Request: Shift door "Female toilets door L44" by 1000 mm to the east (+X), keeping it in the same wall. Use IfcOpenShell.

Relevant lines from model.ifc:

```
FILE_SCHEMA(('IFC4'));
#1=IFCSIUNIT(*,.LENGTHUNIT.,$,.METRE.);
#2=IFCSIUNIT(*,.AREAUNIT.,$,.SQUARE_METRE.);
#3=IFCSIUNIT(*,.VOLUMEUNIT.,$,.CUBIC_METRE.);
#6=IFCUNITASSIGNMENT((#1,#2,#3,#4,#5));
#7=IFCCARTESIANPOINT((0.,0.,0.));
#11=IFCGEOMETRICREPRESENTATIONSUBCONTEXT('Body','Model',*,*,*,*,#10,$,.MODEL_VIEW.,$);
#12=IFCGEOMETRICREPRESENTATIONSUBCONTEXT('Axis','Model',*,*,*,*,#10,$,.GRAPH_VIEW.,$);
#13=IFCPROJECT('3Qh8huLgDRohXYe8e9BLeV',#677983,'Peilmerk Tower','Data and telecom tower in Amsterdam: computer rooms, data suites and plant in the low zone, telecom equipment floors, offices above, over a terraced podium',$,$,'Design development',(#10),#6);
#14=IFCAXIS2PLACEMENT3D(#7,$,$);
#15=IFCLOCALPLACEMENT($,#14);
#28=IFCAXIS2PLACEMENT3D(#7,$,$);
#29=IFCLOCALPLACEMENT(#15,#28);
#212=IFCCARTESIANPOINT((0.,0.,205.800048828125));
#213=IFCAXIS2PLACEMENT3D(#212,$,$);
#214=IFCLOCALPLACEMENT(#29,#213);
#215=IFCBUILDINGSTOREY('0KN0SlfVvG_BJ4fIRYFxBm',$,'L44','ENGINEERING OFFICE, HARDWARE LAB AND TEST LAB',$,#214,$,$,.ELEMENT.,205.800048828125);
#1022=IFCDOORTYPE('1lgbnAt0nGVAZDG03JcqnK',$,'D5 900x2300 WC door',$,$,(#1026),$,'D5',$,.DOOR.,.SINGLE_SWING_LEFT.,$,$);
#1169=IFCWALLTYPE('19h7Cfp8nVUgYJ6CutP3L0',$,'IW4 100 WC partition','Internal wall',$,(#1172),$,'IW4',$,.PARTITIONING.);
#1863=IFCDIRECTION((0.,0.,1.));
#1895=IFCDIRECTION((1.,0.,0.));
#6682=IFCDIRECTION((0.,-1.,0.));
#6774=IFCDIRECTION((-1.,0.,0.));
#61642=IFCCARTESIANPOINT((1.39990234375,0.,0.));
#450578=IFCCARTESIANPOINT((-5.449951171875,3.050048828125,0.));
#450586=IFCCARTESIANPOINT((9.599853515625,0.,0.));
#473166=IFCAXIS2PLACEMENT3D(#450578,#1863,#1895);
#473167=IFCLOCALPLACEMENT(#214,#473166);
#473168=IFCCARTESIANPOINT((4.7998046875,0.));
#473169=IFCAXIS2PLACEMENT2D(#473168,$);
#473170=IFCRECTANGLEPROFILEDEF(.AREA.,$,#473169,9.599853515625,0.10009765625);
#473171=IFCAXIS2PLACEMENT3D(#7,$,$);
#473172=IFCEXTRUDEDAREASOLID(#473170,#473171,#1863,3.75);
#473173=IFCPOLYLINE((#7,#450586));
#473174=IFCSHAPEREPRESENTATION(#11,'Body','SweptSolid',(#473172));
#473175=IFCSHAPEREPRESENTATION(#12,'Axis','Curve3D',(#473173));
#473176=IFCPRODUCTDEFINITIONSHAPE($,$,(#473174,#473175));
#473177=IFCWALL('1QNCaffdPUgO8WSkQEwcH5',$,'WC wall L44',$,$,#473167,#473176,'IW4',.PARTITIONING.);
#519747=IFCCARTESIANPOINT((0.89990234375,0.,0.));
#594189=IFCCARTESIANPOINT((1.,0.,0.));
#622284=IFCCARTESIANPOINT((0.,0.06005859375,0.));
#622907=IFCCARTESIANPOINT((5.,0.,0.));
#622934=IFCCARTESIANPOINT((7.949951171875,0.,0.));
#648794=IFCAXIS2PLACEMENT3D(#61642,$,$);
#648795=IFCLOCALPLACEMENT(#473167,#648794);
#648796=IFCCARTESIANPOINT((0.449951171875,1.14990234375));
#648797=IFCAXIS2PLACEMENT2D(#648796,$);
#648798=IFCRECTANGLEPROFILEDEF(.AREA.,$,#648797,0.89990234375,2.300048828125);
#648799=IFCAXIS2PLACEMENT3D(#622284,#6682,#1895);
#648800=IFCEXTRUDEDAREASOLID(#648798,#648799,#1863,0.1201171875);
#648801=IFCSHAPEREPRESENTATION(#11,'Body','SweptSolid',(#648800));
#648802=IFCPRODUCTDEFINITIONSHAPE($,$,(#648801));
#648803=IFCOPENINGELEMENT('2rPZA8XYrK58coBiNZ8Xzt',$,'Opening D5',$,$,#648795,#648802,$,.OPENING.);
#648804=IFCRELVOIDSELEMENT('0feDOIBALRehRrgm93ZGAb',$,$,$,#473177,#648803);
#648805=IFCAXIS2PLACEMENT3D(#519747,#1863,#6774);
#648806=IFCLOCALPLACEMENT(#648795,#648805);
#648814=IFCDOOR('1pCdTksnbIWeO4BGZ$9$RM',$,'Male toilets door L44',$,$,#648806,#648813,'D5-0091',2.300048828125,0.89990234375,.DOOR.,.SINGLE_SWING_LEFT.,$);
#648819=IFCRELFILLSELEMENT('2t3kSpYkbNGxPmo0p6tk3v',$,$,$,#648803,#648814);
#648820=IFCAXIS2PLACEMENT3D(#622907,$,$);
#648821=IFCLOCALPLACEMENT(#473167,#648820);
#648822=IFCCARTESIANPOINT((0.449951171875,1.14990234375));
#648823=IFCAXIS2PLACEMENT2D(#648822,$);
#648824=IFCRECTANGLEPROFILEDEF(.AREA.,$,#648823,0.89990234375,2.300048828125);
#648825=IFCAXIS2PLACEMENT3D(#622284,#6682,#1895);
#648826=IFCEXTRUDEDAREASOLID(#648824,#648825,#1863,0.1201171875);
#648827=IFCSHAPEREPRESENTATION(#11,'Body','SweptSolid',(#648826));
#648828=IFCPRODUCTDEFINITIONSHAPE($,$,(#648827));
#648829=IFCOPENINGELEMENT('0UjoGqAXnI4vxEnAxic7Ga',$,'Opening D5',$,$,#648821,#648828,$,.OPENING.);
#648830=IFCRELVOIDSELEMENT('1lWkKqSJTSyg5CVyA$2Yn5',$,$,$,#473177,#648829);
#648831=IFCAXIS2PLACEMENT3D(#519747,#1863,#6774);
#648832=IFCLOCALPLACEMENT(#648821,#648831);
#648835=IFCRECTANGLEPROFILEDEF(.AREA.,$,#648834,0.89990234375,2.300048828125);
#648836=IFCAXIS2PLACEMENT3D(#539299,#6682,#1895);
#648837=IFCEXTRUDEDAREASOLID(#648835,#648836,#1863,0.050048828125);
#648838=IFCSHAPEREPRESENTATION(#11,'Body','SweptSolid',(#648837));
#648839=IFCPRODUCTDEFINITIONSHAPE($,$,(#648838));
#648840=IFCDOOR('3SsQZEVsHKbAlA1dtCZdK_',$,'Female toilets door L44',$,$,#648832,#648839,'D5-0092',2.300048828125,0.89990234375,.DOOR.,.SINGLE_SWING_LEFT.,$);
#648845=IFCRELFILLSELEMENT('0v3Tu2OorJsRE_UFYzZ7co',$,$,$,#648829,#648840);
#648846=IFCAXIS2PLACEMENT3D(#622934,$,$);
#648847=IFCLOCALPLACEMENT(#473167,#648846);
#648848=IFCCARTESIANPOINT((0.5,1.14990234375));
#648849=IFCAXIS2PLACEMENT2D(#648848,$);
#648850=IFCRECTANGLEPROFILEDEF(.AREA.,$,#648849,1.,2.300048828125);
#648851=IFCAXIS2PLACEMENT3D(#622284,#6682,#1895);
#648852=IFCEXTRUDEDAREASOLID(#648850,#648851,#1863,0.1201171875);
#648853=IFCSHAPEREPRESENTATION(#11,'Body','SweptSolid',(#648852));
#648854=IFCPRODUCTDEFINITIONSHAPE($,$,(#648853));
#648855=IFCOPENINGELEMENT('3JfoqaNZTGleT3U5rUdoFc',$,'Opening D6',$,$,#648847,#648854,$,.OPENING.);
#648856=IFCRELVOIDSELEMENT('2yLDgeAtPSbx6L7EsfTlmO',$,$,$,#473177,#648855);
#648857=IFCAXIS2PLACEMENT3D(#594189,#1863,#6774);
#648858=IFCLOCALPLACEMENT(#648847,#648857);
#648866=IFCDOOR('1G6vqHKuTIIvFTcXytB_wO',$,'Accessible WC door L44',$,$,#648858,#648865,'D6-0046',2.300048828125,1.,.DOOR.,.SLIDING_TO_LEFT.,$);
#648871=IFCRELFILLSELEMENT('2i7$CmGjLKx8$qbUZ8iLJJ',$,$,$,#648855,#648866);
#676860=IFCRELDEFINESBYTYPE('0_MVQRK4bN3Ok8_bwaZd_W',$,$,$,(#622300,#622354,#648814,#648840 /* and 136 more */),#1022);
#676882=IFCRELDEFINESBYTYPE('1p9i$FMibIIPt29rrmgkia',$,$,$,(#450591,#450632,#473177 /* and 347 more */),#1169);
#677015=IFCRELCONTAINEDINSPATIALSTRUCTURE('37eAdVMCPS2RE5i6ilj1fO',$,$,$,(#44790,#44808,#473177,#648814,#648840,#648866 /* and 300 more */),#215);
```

```python
import ifcopenshell
import ifcopenshell.api.geometry
import ifcopenshell.util.placement
import ifcopenshell.util.unit

model = ifcopenshell.open("model.ifc")
unit_scale = ifcopenshell.util.unit.calculate_unit_scale(model)

door = model.by_guid("3SsQZEVsHKbAlA1dtCZdK_")
opening = door.FillsVoids[0].RelatingOpeningElement
wall = opening.VoidsElements[0].RelatingBuildingElement

wall_matrix = ifcopenshell.util.placement.get_local_placement(wall.ObjectPlacement)
shift = wall_matrix[:3, 0] * 1 / unit_scale
before = ifcopenshell.util.placement.get_local_placement(door.ObjectPlacement)[:3, 3].copy()

# The door is placed relative to its opening, so it follows when the opening moves.
matrix = ifcopenshell.util.placement.get_local_placement(opening.ObjectPlacement)
matrix[:3, 3] += shift
ifcopenshell.api.geometry.edit_object_placement(
    model, product=opening, matrix=matrix, is_si=False, should_transform_children=True
)

after = ifcopenshell.util.placement.get_local_placement(door.ObjectPlacement)[:3, 3]
print("door moved by", (after - before).round(3) + 0.0)

model.write("model_v2.ifc")
```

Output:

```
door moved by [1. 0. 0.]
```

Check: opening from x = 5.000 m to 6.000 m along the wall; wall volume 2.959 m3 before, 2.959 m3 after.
